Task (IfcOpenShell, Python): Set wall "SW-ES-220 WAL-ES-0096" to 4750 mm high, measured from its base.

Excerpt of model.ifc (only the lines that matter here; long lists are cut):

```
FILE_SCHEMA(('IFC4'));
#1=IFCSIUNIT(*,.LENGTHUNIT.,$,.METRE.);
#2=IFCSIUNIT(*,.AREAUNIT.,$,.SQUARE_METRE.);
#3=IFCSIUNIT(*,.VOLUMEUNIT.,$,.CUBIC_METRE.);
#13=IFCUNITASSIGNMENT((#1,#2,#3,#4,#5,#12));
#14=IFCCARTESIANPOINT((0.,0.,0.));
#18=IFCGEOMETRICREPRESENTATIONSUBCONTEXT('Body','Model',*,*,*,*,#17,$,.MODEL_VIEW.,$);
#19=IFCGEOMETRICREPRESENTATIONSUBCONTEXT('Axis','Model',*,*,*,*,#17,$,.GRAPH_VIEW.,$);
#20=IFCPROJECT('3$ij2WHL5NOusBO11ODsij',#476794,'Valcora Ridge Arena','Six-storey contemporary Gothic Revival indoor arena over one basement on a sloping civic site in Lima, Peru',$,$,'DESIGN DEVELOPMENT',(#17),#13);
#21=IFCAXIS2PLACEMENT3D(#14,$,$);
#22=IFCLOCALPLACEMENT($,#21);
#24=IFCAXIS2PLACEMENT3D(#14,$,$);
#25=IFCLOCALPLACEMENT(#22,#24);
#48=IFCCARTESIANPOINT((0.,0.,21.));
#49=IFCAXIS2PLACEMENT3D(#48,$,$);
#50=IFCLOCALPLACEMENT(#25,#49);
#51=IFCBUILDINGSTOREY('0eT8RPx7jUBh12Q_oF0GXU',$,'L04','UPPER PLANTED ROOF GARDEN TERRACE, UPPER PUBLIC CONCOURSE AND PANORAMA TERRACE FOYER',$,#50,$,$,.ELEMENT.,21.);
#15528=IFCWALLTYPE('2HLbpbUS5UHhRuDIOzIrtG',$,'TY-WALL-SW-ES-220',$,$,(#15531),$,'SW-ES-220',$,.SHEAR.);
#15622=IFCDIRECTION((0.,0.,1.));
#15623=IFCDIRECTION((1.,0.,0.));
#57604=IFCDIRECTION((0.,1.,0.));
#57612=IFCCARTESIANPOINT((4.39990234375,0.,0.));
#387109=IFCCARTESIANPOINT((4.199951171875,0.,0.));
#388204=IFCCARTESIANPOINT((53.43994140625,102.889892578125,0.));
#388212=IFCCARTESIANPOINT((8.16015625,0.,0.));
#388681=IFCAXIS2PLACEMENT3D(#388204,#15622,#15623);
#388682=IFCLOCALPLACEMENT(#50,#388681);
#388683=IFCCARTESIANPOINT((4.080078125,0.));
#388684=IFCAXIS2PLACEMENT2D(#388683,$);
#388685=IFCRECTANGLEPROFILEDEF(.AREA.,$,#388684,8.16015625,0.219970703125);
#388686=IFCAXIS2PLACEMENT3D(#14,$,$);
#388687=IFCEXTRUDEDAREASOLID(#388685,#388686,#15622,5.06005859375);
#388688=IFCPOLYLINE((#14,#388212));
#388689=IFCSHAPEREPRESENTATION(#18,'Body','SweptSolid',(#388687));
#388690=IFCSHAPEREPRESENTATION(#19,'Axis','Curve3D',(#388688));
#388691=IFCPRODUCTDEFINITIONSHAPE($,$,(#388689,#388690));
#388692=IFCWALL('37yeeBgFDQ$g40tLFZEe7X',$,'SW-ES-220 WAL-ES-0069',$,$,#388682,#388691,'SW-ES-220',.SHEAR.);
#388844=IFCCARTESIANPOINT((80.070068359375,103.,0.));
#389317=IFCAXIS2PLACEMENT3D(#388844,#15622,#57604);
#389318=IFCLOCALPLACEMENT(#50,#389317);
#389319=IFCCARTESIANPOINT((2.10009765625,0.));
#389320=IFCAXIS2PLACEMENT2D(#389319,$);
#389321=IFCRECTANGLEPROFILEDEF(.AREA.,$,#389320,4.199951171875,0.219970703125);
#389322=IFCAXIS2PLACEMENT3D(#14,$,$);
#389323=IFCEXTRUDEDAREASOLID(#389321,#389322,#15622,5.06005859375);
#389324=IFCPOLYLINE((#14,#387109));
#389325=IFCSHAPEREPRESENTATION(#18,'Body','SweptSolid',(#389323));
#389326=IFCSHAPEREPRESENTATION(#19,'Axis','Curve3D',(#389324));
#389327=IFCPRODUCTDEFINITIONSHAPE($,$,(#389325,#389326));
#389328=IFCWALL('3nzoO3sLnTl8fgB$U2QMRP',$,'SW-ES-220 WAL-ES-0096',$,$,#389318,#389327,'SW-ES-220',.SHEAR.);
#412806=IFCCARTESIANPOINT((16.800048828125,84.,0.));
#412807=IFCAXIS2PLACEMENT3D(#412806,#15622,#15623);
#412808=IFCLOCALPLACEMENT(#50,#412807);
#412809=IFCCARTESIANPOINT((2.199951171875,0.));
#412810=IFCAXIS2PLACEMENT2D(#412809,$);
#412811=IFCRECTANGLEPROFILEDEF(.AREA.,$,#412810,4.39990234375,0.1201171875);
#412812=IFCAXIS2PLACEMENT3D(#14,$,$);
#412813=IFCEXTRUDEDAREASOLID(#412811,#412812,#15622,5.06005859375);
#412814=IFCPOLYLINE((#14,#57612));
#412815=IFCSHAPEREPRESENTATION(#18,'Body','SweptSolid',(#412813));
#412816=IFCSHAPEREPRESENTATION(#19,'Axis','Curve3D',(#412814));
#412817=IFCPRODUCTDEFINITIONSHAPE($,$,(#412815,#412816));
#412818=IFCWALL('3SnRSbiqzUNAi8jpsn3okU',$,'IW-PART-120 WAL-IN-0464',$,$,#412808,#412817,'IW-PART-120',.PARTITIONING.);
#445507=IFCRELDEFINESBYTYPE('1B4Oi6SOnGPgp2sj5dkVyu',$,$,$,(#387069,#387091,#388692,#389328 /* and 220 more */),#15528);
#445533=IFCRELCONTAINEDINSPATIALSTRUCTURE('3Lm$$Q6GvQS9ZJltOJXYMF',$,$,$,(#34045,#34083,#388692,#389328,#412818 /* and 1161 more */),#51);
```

```python
import ifcopenshell
import ifcopenshell.geom
import ifcopenshell.util.representation
import ifcopenshell.util.shape

model = ifcopenshell.open("model.ifc")
settings = ifcopenshell.geom.settings()


def volume(element):
    """Net volume in cubic metres, openings subtracted."""
    shape = ifcopenshell.geom.create_shape(settings, element)
    return ifcopenshell.util.shape.get_volume(shape.geometry)


wall = model.by_id(389328)
before = volume(wall)

body = ifcopenshell.util.representation.get_representation(wall, "Model", "Body")
solid = body.Items[0]
old_height = solid.Depth
solid.Depth = 4.75
after = volume(wall)

print(f"height {old_height:g} -> {solid.Depth:g}, volume {before:.3f} -> {after:.3f} m3")

model.write("model-out.ifc")
```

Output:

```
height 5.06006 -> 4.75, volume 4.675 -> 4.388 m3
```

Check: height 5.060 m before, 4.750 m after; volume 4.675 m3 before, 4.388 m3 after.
